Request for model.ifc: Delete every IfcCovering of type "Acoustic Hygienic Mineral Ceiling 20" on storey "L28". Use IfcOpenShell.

First a look at what the model holds.

```python
import ifcopenshell
import ifcopenshell.util.element

model = ifcopenshell.open("model.ifc")
print(model.schema)
storey = next(s for s in model.by_type("IfcBuildingStorey") if s.Name == "L28")
coverings = [e for e in ifcopenshell.util.element.get_decomposition(storey) if e.is_a("IfcCovering")]
seen = {}
for e in coverings:
    element_type = ifcopenshell.util.element.get_type(e)
    name = element_type.Name if element_type not in (None, e) else None
    seen[name] = seen.get(name, 0) + 1
for name, count in sorted(seen.items(), key=str):
    print(count, "x", name)
```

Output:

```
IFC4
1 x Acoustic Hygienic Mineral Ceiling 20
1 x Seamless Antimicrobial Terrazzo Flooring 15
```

```python
import ifcopenshell
import ifcopenshell.api.root
import ifcopenshell.util.element

model = ifcopenshell.open("model.ifc")

storey = next(s for s in model.by_type("IfcBuildingStorey") if s.Name == "L28")
coverings = [e for e in ifcopenshell.util.element.get_decomposition(storey) if e.is_a("IfcCovering")]
targets = [e for e in coverings if (t := ifcopenshell.util.element.get_type(e)) not in (None, e) and t.Name == "Acoustic Hygienic Mineral Ceiling 20"]

for e in targets:
    ifcopenshell.api.root.remove_product(model, product=e)
print(len(targets), "removed")

model.write("model_edited.ifc")
```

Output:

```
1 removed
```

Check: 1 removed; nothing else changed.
